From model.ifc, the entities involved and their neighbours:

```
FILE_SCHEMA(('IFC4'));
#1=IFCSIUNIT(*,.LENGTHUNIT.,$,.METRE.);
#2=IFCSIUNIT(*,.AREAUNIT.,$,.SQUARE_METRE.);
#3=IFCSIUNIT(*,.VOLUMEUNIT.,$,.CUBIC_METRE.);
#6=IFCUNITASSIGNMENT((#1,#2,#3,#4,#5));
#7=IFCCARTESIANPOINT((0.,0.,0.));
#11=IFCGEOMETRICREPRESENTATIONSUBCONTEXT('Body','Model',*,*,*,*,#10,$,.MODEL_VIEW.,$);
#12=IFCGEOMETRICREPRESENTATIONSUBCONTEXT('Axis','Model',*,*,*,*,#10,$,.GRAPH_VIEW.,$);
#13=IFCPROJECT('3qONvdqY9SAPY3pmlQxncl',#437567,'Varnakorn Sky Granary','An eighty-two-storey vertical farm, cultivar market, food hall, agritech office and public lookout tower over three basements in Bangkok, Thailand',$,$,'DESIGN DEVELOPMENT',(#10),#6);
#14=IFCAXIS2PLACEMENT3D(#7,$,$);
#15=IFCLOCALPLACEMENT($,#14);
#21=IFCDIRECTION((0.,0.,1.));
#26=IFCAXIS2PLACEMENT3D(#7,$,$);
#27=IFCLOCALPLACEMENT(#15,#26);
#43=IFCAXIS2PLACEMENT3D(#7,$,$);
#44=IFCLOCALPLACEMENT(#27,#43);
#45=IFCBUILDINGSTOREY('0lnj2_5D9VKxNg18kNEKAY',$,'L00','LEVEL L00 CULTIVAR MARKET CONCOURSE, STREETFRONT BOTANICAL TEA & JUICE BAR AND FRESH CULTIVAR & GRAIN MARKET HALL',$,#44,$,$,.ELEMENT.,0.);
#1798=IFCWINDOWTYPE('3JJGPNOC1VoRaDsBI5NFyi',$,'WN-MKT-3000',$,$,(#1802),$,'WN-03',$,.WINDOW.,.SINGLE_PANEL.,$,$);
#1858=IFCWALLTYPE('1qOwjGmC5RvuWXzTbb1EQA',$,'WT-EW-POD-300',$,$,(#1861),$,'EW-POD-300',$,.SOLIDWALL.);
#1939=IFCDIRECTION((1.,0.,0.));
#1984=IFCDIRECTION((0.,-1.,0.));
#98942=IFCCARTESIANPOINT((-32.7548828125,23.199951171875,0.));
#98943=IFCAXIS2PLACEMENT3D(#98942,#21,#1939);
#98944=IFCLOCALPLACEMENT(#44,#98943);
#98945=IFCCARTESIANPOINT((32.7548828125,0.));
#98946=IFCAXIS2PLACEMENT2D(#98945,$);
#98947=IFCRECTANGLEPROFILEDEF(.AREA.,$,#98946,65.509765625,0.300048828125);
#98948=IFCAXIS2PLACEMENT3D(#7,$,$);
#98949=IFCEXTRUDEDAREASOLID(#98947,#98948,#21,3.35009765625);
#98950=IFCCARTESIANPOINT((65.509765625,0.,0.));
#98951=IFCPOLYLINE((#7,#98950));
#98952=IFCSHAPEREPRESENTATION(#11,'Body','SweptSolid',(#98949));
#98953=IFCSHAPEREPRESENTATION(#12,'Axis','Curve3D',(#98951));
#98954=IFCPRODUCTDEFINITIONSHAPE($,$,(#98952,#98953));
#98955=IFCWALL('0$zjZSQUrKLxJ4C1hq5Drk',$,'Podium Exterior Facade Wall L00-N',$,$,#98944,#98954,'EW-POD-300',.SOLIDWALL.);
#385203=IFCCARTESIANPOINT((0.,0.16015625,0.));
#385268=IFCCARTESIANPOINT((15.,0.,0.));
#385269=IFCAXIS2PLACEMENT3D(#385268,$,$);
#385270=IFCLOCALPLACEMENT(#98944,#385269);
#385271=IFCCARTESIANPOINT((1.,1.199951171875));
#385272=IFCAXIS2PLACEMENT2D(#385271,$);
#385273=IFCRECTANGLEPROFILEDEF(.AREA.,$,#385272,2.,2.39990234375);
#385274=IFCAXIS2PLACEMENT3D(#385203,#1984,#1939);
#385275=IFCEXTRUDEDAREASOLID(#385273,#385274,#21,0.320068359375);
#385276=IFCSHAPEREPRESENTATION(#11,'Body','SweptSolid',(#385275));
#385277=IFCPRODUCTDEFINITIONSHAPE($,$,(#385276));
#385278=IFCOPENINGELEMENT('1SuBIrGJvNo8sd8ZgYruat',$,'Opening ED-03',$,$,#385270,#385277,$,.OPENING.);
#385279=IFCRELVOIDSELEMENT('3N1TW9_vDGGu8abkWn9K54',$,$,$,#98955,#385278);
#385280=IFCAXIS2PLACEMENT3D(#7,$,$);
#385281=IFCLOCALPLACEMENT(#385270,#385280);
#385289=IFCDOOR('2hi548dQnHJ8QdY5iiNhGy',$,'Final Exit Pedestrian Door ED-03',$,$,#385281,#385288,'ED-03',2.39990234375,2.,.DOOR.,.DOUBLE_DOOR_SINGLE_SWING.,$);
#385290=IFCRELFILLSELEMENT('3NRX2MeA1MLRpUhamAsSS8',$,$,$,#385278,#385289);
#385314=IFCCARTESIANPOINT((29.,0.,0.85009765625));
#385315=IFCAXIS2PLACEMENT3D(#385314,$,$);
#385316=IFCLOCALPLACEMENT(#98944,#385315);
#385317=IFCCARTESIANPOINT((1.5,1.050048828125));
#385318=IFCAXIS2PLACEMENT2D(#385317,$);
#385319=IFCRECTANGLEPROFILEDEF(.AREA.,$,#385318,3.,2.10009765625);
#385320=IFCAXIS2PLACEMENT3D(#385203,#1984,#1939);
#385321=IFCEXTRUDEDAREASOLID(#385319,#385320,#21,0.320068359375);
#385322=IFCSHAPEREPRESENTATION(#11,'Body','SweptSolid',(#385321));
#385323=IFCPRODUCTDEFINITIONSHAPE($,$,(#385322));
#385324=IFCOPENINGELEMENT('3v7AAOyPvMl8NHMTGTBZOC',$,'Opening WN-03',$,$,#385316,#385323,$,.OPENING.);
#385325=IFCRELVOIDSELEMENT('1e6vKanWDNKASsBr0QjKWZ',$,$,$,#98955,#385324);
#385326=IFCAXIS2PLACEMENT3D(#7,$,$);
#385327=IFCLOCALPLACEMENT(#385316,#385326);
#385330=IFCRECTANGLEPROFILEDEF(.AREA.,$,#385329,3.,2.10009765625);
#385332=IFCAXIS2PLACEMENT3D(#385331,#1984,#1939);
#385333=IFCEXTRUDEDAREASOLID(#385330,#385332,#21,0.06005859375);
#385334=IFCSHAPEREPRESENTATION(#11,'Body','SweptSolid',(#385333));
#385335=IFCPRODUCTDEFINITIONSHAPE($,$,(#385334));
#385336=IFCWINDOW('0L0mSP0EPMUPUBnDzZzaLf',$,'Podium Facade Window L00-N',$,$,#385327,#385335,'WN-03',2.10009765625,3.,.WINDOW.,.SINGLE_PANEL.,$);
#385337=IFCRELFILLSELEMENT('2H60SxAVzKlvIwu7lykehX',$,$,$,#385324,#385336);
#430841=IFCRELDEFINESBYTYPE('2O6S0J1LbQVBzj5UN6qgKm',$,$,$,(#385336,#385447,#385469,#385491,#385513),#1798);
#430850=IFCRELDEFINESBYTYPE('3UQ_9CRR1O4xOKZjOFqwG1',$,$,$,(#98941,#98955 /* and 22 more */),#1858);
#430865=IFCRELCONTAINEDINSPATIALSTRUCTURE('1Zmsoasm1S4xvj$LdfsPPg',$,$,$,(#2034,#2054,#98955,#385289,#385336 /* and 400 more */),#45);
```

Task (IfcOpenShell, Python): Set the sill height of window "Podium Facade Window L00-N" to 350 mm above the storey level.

```python
import numpy as np
import ifcopenshell
import ifcopenshell.api.geometry
import ifcopenshell.geom
import ifcopenshell.util.element
import ifcopenshell.util.placement
import ifcopenshell.util.shape
import ifcopenshell.util.unit

model = ifcopenshell.open("model.ifc")
unit_scale = ifcopenshell.util.unit.calculate_unit_scale(model)

window = model.by_guid("0L0mSP0EPMUPUBnDzZzaLf")
opening = window.FillsVoids[0].RelatingOpeningElement
storey = ifcopenshell.util.element.get_container(window, ifc_class="IfcBuildingStorey")
level = ifcopenshell.util.placement.get_local_placement(storey.ObjectPlacement)[2, 3]

# The opening's origin need not be at the sill, so measure its lowest point.
shape = ifcopenshell.geom.create_shape(ifcopenshell.geom.settings(), opening)
bottom = ifcopenshell.util.shape.get_shape_bottom_elevation(shape, shape.geometry) / unit_scale
dz = level + 0.35 - bottom

shift = np.array([0.0, 0.0, dz])
# The window is placed relative to its opening, so it follows when the opening moves.
matrix = ifcopenshell.util.placement.get_local_placement(opening.ObjectPlacement)
matrix[:3, 3] += shift
ifcopenshell.api.geometry.edit_object_placement(
    model, product=opening, matrix=matrix, is_si=False, should_transform_children=True
)

print(f"moved by {dz * unit_scale:+.3f} m")

model.write("model_edited.ifc")
```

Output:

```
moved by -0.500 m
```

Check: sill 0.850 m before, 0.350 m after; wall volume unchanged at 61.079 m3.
